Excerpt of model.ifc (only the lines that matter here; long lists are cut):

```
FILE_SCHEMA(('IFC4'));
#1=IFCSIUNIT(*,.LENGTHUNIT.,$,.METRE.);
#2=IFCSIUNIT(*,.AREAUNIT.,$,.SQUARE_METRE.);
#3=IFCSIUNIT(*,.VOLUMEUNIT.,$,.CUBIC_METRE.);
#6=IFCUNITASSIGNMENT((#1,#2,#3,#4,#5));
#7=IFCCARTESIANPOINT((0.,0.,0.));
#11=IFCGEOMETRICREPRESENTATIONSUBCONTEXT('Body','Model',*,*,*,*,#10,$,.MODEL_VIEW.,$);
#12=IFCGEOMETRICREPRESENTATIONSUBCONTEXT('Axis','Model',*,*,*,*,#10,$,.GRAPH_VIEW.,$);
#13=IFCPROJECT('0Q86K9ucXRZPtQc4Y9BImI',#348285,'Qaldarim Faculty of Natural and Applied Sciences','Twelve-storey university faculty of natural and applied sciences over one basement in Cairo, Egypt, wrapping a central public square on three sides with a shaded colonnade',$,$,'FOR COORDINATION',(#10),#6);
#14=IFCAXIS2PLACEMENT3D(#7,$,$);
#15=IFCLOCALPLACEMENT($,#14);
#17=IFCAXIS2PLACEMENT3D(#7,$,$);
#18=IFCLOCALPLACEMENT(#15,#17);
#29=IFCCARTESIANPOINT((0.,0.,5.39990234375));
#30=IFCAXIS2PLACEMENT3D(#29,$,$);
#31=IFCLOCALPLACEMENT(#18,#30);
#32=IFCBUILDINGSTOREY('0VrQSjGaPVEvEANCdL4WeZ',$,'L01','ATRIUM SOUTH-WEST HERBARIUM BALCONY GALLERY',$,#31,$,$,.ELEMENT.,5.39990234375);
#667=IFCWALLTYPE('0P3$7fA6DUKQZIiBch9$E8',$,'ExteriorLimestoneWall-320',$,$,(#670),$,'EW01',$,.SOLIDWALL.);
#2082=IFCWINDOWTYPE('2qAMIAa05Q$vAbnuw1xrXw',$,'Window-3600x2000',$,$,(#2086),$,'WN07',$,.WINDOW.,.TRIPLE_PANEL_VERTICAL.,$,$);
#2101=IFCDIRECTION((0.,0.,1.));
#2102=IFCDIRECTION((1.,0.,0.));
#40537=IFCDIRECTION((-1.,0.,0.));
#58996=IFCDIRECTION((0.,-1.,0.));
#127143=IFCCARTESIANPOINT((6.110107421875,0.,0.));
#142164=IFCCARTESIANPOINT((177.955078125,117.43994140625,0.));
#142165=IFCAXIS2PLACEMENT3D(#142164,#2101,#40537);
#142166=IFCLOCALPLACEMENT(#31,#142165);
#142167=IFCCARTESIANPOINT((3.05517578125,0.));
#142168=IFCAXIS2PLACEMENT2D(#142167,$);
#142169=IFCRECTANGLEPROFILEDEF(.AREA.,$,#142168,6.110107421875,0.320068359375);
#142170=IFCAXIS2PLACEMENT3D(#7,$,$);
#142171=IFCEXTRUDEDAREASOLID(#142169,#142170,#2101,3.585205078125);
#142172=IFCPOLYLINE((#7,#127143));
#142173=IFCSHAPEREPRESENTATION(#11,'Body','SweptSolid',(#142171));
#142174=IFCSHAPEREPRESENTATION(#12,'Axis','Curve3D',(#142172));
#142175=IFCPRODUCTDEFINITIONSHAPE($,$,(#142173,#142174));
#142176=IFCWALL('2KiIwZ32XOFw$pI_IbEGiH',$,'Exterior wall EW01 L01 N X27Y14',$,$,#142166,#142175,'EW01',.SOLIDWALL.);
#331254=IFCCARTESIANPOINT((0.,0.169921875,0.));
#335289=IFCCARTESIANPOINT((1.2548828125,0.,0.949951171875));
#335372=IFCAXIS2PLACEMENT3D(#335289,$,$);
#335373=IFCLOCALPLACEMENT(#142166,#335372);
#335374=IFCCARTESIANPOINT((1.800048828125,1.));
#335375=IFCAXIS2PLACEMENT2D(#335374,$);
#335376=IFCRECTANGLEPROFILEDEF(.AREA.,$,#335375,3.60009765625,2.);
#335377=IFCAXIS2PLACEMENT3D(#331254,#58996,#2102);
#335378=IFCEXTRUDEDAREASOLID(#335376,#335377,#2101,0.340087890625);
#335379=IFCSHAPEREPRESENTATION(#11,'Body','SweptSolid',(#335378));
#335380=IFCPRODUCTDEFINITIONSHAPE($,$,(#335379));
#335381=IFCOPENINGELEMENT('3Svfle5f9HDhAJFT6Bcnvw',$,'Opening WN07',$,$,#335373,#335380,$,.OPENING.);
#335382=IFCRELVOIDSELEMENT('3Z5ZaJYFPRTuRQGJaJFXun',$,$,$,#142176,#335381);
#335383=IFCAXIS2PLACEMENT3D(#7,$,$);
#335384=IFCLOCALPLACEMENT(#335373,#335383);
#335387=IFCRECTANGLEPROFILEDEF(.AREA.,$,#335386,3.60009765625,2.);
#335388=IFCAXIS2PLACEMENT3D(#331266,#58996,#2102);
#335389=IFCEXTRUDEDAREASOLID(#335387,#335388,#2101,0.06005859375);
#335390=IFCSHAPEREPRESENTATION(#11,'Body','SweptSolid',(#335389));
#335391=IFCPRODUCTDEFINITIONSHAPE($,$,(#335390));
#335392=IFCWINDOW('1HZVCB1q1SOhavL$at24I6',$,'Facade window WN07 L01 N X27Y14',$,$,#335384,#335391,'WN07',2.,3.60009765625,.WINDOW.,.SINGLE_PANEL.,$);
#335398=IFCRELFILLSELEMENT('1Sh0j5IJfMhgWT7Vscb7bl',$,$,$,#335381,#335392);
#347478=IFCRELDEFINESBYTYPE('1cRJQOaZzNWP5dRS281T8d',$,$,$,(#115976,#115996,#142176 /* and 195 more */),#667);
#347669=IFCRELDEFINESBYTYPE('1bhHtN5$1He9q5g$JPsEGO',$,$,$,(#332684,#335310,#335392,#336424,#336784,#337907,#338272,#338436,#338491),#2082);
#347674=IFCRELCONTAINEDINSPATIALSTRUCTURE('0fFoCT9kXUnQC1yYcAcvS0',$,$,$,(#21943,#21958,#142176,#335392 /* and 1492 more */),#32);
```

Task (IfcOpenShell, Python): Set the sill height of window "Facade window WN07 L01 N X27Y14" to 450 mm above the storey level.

```python
import numpy as np
import ifcopenshell
import ifcopenshell.api.geometry
import ifcopenshell.geom
import ifcopenshell.util.element
import ifcopenshell.util.placement
import ifcopenshell.util.shape
import ifcopenshell.util.unit

model = ifcopenshell.open("model.ifc")
unit_scale = ifcopenshell.util.unit.calculate_unit_scale(model)

window = model.by_guid("1HZVCB1q1SOhavL$at24I6")
opening = window.FillsVoids[0].RelatingOpeningElement
storey = ifcopenshell.util.element.get_container(window, ifc_class="IfcBuildingStorey")
level = ifcopenshell.util.placement.get_local_placement(storey.ObjectPlacement)[2, 3]

# The opening's origin need not be at the sill, so measure its lowest point.
shape = ifcopenshell.geom.create_shape(ifcopenshell.geom.settings(), opening)
bottom = ifcopenshell.util.shape.get_shape_bottom_elevation(shape, shape.geometry) / unit_scale
dz = level + 0.45 - bottom

shift = np.array([0.0, 0.0, dz])
# The window is placed relative to its opening, so it follows when the opening moves.
matrix = ifcopenshell.util.placement.get_local_placement(opening.ObjectPlacement)
matrix[:3, 3] += shift
ifcopenshell.api.geometry.edit_object_placement(
    model, product=opening, matrix=matrix, is_si=False, should_transform_children=True
)

print(f"moved by {dz * unit_scale:+.3f} m")

model.write("model_rev.ifc")
```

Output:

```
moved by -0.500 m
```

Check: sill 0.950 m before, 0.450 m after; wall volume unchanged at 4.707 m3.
